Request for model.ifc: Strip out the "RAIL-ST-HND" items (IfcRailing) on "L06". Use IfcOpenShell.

First a look at what the model holds.

```python
import ifcopenshell
import ifcopenshell.util.element

model = ifcopenshell.open("model.ifc")
print(model.schema)
storey = next(s for s in model.by_type("IfcBuildingStorey") if s.Name == "L06")
railings = [e for e in ifcopenshell.util.element.get_decomposition(storey) if e.is_a("IfcRailing")]
seen = {}
for e in railings:
    element_type = ifcopenshell.util.element.get_type(e)
    name = element_type.Name if element_type not in (None, e) else None
    seen[name] = seen.get(name, 0) + 1
for name, count in sorted(seen.items(), key=str):
    print(count, "x", name)
```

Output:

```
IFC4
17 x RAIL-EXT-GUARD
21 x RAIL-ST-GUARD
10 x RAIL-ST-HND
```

```python
import ifcopenshell
import ifcopenshell.api.root
import ifcopenshell.util.element

model = ifcopenshell.open("model.ifc")

storey = next(s for s in model.by_type("IfcBuildingStorey") if s.Name == "L06")
railings = [e for e in ifcopenshell.util.element.get_decomposition(storey) if e.is_a("IfcRailing")]
targets = [e for e in railings if (t := ifcopenshell.util.element.get_type(e)) not in (None, e) and t.Name == "RAIL-ST-HND"]

for e in targets:
    ifcopenshell.api.root.remove_product(model, product=e)
print(len(targets), "removed")

model.write("model_rev.ifc")
```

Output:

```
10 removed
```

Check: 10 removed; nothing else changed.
